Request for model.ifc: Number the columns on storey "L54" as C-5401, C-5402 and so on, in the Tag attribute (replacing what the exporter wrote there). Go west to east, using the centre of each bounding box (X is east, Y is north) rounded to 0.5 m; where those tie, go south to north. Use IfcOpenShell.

First a look at what the model holds.

```python
import ifcopenshell
import ifcopenshell.util.element
import ifcopenshell.util.placement

model = ifcopenshell.open("model.ifc")
print(model.schema)
storey = next(s for s in model.by_type("IfcBuildingStorey") if s.Name == "L54")
columns = [e for e in ifcopenshell.util.element.get_decomposition(storey) if e.is_a("IfcColumn")]
for e in sorted(columns, key=lambda e: e.id()):
    origin = ifcopenshell.util.placement.get_local_placement(e.ObjectPlacement)[:3, 3]
    print(e.id(), e.Tag, e.Name, origin.round(2) + 0.0, sep=" | ")
```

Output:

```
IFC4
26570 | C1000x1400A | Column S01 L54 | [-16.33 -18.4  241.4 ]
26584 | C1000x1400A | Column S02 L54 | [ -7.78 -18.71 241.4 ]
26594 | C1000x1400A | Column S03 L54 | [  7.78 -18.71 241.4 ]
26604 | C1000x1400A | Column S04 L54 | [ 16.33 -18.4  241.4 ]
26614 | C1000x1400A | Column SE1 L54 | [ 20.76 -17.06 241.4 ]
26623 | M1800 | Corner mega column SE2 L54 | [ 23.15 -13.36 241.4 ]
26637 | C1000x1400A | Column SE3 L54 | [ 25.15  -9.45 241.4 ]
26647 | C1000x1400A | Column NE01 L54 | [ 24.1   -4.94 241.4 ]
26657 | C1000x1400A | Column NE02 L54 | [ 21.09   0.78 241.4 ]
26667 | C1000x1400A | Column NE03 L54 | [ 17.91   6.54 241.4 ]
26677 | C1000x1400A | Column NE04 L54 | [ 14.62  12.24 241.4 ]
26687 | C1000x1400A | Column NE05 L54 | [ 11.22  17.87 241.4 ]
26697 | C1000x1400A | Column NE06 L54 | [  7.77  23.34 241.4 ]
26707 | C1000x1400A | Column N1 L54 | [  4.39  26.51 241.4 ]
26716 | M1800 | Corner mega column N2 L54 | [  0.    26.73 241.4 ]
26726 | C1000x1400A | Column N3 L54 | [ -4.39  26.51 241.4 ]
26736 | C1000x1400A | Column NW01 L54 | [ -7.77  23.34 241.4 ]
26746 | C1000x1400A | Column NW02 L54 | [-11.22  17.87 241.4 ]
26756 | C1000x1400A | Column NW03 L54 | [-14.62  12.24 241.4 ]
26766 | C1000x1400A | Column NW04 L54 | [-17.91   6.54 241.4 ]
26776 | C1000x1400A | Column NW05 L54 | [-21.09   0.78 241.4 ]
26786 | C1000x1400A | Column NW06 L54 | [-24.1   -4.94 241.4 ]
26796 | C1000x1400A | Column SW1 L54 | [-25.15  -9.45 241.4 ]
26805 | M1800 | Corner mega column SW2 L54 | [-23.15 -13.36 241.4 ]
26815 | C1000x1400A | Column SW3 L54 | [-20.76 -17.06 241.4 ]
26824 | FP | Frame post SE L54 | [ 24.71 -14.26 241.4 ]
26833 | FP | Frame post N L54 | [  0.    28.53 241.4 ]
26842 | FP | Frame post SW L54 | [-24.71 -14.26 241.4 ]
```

```python
import ifcopenshell
import ifcopenshell.geom
import ifcopenshell.util.element
import ifcopenshell.util.shape

model = ifcopenshell.open("model.ifc")
settings = ifcopenshell.geom.settings()
settings.set("use-world-coords", True)


def centre(element):
    shape = ifcopenshell.geom.create_shape(settings, element)
    return ifcopenshell.util.shape.get_bbox_centroid(shape.geometry)


storey = next(s for s in model.by_type("IfcBuildingStorey") if s.Name == "L54")
columns = [e for e in ifcopenshell.util.element.get_decomposition(storey) if e.is_a("IfcColumn")]

# Insertion points can sit at a corner or the storey origin, so sort by the geometry (in metres).
centres = {e: centre(e) for e in columns}
columns.sort(key=lambda e: (round(centres[e][0] / 0.5), centres[e][1]))

for i, e in enumerate(columns, start=1):
    number = f"C-54{i:02d}"
    e.Tag = number
    print(e.id(), number)

model.write("model_v2.ifc")
```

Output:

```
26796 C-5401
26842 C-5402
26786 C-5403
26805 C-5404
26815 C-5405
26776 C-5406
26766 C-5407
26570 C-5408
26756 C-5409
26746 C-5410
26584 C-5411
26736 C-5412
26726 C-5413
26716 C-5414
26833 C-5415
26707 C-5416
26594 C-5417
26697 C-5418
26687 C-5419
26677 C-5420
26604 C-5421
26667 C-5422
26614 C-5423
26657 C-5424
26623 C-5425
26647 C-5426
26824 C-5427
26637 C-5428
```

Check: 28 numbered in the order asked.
